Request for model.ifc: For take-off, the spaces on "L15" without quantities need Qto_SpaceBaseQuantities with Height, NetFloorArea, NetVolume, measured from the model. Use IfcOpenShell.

First a look at what the model holds.

```python
import ifcopenshell
import ifcopenshell.util.element
import ifcopenshell.util.unit

model = ifcopenshell.open("model.ifc")
print(model.schema)
for unit_type in ("LENGTHUNIT", "AREAUNIT", "VOLUMEUNIT"):
    print(unit_type, ifcopenshell.util.unit.calculate_unit_scale(model, unit_type))
storey = next(s for s in model.by_type("IfcBuildingStorey") if s.Name == "L15")
spaces = [e for e in ifcopenshell.util.element.get_decomposition(storey) if e.is_a("IfcSpace")]
for e in sorted(spaces, key=lambda e: e.id()):
    print(e.id(), e.is_a(), e.Name, list(ifcopenshell.util.element.get_psets(e, qtos_only=True)), sep=" | ")
```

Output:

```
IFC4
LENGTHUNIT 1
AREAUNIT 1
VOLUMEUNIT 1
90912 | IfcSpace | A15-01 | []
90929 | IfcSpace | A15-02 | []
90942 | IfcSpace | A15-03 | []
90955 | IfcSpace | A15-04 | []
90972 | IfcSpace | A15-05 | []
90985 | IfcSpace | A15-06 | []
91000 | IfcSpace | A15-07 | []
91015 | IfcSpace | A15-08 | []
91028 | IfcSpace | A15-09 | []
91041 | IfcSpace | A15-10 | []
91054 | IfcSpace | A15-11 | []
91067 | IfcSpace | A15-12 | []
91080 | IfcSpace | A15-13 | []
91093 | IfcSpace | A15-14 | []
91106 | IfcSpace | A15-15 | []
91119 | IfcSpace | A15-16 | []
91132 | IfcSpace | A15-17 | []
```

```python
import ifcopenshell
import ifcopenshell.api.pset
import ifcopenshell.geom
import ifcopenshell.util.element
import ifcopenshell.util.shape
import ifcopenshell.util.unit

model = ifcopenshell.open("model.ifc")
unit_scale = ifcopenshell.util.unit.calculate_unit_scale(model)
area_scale = ifcopenshell.util.unit.calculate_unit_scale(model, "AREAUNIT")
volume_scale = ifcopenshell.util.unit.calculate_unit_scale(model, "VOLUMEUNIT")
settings = ifcopenshell.geom.settings()

storey = next(s for s in model.by_type("IfcBuildingStorey") if s.Name == "L15")
spaces = [e for e in ifcopenshell.util.element.get_decomposition(storey) if e.is_a("IfcSpace")]

for e in sorted(spaces, key=lambda e: e.id()):
    if ifcopenshell.util.element.get_psets(e, qtos_only=True, should_inherit=False):
        continue
    # Geometry comes back in metres, in the element's own axes.
    shape = ifcopenshell.geom.create_shape(settings, e)
    values = {
        "Height": ifcopenshell.util.shape.get_z(shape.geometry) / unit_scale,
        "NetFloorArea": ifcopenshell.util.shape.get_footprint_area(shape.geometry) / area_scale,
        "NetVolume": ifcopenshell.util.shape.get_volume(shape.geometry) / volume_scale,
    }
    qto = ifcopenshell.api.pset.add_qto(model, product=e, name="Qto_SpaceBaseQuantities")
    ifcopenshell.api.pset.edit_qto(model, qto=qto, properties=values)
    print(e.id(), {k: round(v, 3) for k, v in values.items()})

model.write("model-out.ifc")
```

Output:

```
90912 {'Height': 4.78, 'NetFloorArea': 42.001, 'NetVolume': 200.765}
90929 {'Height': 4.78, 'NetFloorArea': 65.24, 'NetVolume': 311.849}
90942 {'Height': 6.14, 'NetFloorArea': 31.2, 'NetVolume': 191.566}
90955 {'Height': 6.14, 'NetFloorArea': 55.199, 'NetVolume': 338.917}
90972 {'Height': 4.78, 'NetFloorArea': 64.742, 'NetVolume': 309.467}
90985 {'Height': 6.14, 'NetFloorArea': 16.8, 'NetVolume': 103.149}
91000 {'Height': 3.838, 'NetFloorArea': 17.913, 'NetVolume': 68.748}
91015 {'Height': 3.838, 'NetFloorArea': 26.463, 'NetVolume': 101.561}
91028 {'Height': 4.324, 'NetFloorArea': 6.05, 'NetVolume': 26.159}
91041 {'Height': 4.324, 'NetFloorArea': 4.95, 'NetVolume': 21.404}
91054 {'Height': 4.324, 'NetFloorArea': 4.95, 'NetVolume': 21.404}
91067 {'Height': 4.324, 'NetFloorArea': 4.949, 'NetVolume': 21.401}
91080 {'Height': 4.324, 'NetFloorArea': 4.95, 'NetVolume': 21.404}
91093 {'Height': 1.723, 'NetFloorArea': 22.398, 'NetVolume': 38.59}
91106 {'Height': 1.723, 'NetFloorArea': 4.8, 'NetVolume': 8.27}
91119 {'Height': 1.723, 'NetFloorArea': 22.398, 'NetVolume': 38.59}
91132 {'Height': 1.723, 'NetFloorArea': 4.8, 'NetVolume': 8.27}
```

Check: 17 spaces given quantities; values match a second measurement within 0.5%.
